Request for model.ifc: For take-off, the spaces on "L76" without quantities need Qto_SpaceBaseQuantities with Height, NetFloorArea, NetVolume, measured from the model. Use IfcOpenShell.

First a look at what the model holds.

```python
import ifcopenshell
import ifcopenshell.util.element
import ifcopenshell.util.unit

model = ifcopenshell.open("model.ifc")
print(model.schema)
for unit_type in ("LENGTHUNIT", "AREAUNIT", "VOLUMEUNIT"):
    print(unit_type, ifcopenshell.util.unit.calculate_unit_scale(model, unit_type))
storey = next(s for s in model.by_type("IfcBuildingStorey") if s.Name == "L76")
spaces = [e for e in ifcopenshell.util.element.get_decomposition(storey) if e.is_a("IfcSpace")]
for e in sorted(spaces, key=lambda e: e.id()):
    print(e.id(), e.is_a(), e.Name, list(ifcopenshell.util.element.get_psets(e, qtos_only=True)), sep=" | ")
```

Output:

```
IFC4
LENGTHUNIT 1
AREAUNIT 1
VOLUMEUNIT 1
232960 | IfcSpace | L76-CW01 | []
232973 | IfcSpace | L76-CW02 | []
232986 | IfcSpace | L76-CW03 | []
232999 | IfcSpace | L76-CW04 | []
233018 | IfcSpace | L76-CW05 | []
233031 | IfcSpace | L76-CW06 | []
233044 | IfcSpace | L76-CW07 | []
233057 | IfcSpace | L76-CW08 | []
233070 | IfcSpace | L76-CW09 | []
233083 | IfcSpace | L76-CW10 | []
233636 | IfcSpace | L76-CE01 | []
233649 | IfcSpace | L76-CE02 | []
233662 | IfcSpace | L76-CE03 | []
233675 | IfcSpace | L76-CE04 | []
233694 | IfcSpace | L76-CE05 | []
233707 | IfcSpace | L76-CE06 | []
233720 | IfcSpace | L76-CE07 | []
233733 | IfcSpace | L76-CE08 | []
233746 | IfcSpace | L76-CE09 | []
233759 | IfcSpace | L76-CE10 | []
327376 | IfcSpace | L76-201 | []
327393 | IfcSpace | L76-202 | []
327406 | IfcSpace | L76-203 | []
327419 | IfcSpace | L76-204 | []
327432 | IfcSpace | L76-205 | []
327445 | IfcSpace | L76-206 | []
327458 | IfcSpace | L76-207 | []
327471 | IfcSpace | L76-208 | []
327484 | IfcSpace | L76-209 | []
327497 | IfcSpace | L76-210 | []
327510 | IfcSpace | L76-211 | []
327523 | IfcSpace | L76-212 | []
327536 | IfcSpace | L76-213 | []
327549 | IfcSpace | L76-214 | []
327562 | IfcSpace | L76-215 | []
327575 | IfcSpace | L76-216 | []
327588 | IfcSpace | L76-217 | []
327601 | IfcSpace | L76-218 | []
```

```python
import ifcopenshell
import ifcopenshell.api.pset
import ifcopenshell.geom
import ifcopenshell.util.element
import ifcopenshell.util.shape
import ifcopenshell.util.unit

model = ifcopenshell.open("model.ifc")
unit_scale = ifcopenshell.util.unit.calculate_unit_scale(model)
area_scale = ifcopenshell.util.unit.calculate_unit_scale(model, "AREAUNIT")
volume_scale = ifcopenshell.util.unit.calculate_unit_scale(model, "VOLUMEUNIT")
settings = ifcopenshell.geom.settings()

storey = next(s for s in model.by_type("IfcBuildingStorey") if s.Name == "L76")
spaces = [e for e in ifcopenshell.util.element.get_decomposition(storey) if e.is_a("IfcSpace")]

for e in sorted(spaces, key=lambda e: e.id()):
    if ifcopenshell.util.element.get_psets(e, qtos_only=True, should_inherit=False):
        continue
    # Geometry comes back in metres, in the element's own axes.
    shape = ifcopenshell.geom.create_shape(settings, e)
    values = {
        "Height": ifcopenshell.util.shape.get_z(shape.geometry) / unit_scale,
        "NetFloorArea": ifcopenshell.util.shape.get_footprint_area(shape.geometry) / area_scale,
        "NetVolume": ifcopenshell.util.shape.get_volume(shape.geometry) / volume_scale,
    }
    qto = ifcopenshell.api.pset.add_qto(model, product=e, name="Qto_SpaceBaseQuantities")
    ifcopenshell.api.pset.edit_qto(model, qto=qto, properties=values)
    print(e.id(), {k: round(v, 3) for k, v in values.items()})

model.write("model-out.ifc")
```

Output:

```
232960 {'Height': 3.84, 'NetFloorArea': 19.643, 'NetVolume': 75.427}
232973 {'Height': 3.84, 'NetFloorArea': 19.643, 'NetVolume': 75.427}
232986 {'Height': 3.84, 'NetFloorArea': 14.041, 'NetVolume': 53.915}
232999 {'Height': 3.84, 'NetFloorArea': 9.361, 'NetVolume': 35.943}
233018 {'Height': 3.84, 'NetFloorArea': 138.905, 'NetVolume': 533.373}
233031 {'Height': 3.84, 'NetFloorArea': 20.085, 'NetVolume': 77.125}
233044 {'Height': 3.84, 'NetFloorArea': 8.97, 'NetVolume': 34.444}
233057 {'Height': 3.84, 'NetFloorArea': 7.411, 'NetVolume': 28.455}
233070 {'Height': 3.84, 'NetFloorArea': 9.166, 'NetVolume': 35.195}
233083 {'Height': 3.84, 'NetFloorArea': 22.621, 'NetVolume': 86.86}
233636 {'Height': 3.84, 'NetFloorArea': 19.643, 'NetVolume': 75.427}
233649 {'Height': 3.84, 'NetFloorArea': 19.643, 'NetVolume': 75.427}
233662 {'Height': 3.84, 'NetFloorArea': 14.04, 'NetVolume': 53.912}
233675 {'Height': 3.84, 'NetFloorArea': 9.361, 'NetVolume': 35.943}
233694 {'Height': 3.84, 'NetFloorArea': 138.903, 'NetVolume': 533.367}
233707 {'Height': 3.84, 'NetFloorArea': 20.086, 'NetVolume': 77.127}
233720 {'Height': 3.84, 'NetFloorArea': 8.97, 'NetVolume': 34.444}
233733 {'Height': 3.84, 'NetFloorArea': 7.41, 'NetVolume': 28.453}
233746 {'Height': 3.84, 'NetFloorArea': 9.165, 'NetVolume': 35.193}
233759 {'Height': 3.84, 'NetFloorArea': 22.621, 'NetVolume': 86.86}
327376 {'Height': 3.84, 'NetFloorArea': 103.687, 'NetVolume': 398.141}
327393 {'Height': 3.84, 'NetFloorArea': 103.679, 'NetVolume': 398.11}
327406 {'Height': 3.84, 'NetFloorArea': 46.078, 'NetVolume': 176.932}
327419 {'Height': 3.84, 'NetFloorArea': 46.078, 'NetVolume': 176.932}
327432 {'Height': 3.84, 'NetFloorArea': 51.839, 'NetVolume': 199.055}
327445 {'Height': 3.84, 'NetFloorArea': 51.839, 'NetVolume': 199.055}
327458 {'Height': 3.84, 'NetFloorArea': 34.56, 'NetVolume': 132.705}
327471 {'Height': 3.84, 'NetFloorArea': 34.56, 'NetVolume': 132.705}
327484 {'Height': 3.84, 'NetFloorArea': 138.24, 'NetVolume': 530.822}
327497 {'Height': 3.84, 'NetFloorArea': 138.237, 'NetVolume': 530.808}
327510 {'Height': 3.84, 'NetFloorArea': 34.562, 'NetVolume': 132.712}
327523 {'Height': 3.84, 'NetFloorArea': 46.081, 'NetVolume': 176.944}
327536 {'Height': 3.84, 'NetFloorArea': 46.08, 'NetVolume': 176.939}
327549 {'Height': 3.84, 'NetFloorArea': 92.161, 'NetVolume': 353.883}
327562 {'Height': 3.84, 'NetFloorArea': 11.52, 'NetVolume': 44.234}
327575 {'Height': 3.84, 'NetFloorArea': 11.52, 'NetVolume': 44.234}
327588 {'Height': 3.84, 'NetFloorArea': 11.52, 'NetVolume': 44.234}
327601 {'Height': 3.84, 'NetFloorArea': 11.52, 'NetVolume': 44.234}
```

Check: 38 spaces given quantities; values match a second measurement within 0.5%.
